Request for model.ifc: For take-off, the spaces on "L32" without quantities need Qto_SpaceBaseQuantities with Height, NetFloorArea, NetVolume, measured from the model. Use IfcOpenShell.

First a look at what the model holds.

```python
import ifcopenshell
import ifcopenshell.util.element
import ifcopenshell.util.unit

model = ifcopenshell.open("model.ifc")
print(model.schema)
for unit_type in ("LENGTHUNIT", "AREAUNIT", "VOLUMEUNIT"):
    print(unit_type, ifcopenshell.util.unit.calculate_unit_scale(model, unit_type))
storey = next(s for s in model.by_type("IfcBuildingStorey") if s.Name == "L32")
spaces = [e for e in ifcopenshell.util.element.get_decomposition(storey) if e.is_a("IfcSpace")]
for e in sorted(spaces, key=lambda e: e.id()):
    print(e.id(), e.is_a(), e.Name, list(ifcopenshell.util.element.get_psets(e, qtos_only=True)), sep=" | ")
```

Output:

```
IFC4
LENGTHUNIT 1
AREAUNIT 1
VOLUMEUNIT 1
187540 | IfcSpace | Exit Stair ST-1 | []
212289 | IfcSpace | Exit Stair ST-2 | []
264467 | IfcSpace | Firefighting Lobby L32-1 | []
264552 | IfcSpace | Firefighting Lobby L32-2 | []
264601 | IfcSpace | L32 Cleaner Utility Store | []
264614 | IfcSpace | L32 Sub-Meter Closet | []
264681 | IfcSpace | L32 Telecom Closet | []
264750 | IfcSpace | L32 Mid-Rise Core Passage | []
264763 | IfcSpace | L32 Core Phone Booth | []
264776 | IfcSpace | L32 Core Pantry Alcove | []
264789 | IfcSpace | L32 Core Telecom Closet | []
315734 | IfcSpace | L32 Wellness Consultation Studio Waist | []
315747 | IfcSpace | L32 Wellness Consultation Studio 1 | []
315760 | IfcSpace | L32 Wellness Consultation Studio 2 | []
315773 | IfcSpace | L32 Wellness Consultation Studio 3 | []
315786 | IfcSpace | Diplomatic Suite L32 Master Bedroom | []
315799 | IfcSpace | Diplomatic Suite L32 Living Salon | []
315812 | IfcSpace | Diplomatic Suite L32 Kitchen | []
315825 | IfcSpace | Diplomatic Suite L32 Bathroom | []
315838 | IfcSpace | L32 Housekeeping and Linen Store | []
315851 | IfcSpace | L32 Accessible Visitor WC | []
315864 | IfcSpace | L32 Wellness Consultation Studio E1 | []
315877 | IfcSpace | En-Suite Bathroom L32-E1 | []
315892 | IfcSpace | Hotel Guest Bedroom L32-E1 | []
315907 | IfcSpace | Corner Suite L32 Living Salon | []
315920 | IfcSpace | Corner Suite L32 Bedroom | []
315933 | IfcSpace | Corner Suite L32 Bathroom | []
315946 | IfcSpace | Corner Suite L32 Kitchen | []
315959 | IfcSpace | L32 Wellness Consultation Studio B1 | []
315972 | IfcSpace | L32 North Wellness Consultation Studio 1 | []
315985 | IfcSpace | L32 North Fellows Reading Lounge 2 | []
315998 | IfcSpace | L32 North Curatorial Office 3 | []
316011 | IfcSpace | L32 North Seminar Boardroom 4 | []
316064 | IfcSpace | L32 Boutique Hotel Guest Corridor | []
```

```python
import ifcopenshell
import ifcopenshell.api.pset
import ifcopenshell.geom
import ifcopenshell.util.element
import ifcopenshell.util.shape
import ifcopenshell.util.unit

model = ifcopenshell.open("model.ifc")
unit_scale = ifcopenshell.util.unit.calculate_unit_scale(model)
area_scale = ifcopenshell.util.unit.calculate_unit_scale(model, "AREAUNIT")
volume_scale = ifcopenshell.util.unit.calculate_unit_scale(model, "VOLUMEUNIT")
settings = ifcopenshell.geom.settings()

storey = next(s for s in model.by_type("IfcBuildingStorey") if s.Name == "L32")
spaces = [e for e in ifcopenshell.util.element.get_decomposition(storey) if e.is_a("IfcSpace")]

for e in sorted(spaces, key=lambda e: e.id()):
    if ifcopenshell.util.element.get_psets(e, qtos_only=True, should_inherit=False):
        continue
    # Geometry comes back in metres, in the element's own axes.
    shape = ifcopenshell.geom.create_shape(settings, e)
    values = {
        "Height": ifcopenshell.util.shape.get_z(shape.geometry) / unit_scale,
        "NetFloorArea": ifcopenshell.util.shape.get_footprint_area(shape.geometry) / area_scale,
        "NetVolume": ifcopenshell.util.shape.get_volume(shape.geometry) / volume_scale,
    }
    qto = ifcopenshell.api.pset.add_qto(model, product=e, name="Qto_SpaceBaseQuantities")
    ifcopenshell.api.pset.edit_qto(model, qto=qto, properties=values)
    print(e.id(), {k: round(v, 3) for k, v in values.items()})

model.write("model-out.ifc")
```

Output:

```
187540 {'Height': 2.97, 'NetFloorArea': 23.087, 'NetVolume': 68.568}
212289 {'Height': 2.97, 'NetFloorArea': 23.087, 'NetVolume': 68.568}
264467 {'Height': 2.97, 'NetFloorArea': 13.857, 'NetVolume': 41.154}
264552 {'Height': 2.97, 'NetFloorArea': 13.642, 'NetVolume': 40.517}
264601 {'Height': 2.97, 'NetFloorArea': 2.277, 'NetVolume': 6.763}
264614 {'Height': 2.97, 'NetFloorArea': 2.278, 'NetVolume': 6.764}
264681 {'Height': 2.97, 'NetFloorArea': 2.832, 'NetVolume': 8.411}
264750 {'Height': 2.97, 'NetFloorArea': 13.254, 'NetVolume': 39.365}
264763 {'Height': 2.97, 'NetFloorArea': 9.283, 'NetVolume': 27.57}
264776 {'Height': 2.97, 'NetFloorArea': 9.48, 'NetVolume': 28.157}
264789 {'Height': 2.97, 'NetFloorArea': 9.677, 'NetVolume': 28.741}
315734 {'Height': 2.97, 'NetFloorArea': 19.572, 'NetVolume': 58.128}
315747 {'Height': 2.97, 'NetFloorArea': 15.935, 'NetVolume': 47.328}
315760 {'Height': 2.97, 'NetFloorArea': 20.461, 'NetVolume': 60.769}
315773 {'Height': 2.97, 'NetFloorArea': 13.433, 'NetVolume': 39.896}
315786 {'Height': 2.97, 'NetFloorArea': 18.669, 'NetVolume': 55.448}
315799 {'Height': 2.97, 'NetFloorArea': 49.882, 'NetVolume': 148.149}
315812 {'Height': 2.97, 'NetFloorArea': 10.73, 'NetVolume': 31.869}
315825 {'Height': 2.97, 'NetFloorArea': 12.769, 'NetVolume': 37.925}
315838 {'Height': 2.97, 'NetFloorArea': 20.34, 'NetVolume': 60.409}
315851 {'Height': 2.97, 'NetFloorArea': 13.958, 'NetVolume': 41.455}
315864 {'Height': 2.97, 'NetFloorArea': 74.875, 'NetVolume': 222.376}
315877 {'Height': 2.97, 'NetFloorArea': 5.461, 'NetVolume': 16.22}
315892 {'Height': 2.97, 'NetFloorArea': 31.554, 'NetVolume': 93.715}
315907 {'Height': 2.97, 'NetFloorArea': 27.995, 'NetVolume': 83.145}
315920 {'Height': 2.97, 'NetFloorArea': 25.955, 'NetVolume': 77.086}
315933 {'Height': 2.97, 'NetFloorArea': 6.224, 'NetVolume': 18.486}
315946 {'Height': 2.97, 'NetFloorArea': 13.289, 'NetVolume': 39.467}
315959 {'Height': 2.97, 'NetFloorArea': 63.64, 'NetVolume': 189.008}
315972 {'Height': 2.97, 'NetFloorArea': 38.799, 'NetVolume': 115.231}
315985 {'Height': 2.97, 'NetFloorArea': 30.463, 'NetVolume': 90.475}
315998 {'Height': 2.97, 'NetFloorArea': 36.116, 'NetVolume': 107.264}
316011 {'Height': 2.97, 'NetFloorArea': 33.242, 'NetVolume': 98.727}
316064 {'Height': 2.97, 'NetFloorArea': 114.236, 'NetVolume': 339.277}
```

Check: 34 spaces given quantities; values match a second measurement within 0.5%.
